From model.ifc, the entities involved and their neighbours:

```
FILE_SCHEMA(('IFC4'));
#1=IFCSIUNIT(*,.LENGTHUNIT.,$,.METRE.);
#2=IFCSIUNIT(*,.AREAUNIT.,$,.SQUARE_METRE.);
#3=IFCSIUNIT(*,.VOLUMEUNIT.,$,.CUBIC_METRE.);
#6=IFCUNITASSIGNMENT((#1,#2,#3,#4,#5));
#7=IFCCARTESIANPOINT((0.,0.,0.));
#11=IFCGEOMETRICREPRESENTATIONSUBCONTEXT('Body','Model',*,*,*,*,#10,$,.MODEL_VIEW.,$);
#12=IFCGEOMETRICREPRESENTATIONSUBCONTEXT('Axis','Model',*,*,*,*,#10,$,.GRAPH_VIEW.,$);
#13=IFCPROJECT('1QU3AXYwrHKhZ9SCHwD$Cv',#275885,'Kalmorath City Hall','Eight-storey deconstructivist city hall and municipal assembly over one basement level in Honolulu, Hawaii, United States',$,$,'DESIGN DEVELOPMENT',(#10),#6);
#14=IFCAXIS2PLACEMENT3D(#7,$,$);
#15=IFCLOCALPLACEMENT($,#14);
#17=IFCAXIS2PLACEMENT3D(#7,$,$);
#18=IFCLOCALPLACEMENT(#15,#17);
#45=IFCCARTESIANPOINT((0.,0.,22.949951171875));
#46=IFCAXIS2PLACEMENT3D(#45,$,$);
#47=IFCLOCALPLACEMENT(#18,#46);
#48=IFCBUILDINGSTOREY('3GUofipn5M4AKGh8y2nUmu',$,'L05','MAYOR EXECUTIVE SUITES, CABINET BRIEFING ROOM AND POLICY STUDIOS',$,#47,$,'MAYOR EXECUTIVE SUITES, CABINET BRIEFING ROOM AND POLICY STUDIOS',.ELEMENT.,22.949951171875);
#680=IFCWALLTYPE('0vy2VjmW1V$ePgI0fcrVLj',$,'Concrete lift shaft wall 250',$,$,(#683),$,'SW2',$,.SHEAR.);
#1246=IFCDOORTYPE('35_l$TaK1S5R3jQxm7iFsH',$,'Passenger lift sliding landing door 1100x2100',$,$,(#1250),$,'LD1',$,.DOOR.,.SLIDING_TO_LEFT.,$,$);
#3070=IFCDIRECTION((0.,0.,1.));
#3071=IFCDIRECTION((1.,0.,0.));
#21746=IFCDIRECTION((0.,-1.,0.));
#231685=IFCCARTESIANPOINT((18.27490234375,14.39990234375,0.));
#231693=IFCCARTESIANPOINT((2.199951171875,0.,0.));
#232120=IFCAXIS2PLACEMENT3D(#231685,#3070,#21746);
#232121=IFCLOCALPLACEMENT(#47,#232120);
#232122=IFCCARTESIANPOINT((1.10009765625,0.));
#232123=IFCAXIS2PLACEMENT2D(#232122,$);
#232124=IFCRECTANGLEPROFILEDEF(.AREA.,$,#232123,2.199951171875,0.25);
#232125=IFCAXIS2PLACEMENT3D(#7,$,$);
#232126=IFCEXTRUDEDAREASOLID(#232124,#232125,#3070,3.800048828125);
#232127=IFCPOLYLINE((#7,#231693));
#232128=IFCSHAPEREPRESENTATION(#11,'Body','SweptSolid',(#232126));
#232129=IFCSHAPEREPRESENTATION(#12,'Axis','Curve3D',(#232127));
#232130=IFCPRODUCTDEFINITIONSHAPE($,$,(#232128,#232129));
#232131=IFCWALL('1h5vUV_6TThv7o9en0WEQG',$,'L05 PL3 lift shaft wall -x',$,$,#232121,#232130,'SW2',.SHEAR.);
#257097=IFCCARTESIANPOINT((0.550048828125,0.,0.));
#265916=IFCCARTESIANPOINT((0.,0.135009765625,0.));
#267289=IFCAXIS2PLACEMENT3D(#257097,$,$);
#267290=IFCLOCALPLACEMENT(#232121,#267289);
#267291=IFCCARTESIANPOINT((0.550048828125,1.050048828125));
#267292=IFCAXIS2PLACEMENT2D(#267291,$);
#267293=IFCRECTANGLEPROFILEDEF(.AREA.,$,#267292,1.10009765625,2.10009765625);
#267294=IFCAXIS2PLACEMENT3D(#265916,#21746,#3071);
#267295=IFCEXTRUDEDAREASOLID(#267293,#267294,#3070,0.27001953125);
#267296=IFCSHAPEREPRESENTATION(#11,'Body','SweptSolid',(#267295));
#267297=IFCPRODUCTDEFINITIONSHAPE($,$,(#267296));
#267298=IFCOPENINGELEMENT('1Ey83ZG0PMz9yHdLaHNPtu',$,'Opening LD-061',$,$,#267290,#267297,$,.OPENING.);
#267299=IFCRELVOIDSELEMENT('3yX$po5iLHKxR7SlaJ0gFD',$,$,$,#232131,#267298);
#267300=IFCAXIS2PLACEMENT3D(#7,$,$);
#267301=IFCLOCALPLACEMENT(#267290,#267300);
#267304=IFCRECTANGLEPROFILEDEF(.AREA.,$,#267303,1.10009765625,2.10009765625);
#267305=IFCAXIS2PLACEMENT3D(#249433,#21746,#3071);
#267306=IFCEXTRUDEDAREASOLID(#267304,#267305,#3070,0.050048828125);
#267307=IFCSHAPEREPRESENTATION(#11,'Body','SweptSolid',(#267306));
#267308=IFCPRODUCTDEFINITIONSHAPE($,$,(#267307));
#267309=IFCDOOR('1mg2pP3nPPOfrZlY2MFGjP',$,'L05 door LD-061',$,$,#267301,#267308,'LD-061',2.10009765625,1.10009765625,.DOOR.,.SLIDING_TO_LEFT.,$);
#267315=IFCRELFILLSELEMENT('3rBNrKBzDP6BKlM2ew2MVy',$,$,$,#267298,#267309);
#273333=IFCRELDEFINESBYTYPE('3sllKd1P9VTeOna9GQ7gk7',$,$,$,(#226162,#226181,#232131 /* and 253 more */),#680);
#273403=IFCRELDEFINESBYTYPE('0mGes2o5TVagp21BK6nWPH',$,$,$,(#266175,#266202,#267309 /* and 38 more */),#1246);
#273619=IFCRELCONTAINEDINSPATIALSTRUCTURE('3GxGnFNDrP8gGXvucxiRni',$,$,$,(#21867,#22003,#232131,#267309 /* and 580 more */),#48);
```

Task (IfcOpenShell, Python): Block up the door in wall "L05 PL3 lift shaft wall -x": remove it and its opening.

```python
import ifcopenshell
import ifcopenshell.api.feature
import ifcopenshell.api.root
import ifcopenshell.geom
import ifcopenshell.util.shape

model = ifcopenshell.open("model.ifc")
settings = ifcopenshell.geom.settings()


def volume(element):
    """Net volume in cubic metres, openings subtracted."""
    shape = ifcopenshell.geom.create_shape(settings, element)
    return ifcopenshell.util.shape.get_volume(shape.geometry)


door = model.by_guid("1mg2pP3nPPOfrZlY2MFGjP")
opening = door.FillsVoids[0].RelatingOpeningElement
wall = opening.VoidsElements[0].RelatingBuildingElement
before = volume(wall)

ifcopenshell.api.root.remove_product(model, product=door)
ifcopenshell.api.feature.remove_feature(model, feature=opening)

after = volume(wall)

print(f"wall volume {before:.3f} -> {after:.3f} m3")

model.write("model-out.ifc")
```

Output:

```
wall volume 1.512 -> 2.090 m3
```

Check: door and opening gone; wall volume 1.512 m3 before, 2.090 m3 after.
